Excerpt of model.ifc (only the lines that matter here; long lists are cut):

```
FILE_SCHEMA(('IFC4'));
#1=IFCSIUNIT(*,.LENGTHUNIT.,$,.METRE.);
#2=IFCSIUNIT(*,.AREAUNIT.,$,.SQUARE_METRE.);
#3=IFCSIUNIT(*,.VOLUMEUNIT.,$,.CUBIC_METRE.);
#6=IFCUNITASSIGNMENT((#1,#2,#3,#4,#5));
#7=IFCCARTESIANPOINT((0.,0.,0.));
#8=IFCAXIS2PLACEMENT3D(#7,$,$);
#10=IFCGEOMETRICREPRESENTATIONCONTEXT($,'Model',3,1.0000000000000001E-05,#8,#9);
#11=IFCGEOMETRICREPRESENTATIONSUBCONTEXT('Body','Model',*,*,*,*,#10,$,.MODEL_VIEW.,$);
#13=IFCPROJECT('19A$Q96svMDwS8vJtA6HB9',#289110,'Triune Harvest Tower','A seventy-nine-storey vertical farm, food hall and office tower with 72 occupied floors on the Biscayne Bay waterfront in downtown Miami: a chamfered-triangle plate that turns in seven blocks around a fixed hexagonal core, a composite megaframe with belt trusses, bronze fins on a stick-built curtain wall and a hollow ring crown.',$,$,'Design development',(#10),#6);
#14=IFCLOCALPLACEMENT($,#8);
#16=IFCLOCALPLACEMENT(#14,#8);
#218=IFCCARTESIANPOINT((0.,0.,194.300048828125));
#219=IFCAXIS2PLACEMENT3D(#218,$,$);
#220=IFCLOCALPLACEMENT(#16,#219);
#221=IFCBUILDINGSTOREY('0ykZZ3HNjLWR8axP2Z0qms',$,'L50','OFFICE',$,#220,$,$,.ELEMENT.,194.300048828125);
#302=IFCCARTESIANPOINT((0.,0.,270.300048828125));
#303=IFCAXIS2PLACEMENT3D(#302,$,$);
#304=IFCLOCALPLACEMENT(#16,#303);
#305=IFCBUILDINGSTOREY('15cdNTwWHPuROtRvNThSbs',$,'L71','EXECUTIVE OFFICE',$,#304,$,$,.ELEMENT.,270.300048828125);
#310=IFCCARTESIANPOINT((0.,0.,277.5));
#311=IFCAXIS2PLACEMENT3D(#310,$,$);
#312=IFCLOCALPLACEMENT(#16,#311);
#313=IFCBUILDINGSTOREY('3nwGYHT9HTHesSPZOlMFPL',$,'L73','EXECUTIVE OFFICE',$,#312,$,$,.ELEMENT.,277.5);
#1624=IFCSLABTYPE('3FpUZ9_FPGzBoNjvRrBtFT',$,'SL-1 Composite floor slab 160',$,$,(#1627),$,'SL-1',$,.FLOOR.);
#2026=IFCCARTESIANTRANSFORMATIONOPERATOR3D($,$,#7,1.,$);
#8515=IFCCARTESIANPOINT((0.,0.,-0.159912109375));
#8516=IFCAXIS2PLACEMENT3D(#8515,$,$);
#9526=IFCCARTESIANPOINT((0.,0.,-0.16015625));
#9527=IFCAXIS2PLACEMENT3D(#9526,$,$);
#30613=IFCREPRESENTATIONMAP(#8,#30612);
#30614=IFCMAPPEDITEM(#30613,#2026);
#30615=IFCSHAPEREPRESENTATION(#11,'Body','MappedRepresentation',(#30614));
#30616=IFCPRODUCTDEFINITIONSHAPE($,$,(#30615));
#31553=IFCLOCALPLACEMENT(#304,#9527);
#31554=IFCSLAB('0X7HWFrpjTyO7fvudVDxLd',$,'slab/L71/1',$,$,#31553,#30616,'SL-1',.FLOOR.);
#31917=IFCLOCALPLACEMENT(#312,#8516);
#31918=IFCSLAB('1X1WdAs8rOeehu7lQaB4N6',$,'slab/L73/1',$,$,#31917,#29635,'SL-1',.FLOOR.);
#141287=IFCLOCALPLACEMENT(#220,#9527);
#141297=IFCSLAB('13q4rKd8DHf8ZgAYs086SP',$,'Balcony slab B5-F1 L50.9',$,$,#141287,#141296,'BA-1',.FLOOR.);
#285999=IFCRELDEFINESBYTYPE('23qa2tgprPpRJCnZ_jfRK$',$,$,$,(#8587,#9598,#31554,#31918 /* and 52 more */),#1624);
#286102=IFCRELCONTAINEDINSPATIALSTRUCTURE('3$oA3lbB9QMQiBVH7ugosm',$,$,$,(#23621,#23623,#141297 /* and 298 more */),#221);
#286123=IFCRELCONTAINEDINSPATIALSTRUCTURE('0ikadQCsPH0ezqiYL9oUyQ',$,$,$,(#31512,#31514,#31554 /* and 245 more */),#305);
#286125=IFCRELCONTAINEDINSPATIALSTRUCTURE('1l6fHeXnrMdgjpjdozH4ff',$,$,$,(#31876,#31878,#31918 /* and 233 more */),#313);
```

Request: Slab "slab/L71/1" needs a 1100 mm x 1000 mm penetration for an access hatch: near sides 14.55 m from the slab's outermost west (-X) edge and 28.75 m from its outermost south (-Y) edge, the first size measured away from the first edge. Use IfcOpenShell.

```python
import numpy as np
import ifcopenshell
import ifcopenshell.api.feature
import ifcopenshell.api.geometry
import ifcopenshell.api.root
import ifcopenshell.geom
import ifcopenshell.util.placement
import ifcopenshell.util.representation
import ifcopenshell.util.shape
import ifcopenshell.util.unit

model = ifcopenshell.open("model.ifc")
unit_scale = ifcopenshell.util.unit.calculate_unit_scale(model)
settings = ifcopenshell.geom.settings()


def volume(element):
    """Net volume in cubic metres, openings subtracted."""
    shape = ifcopenshell.geom.create_shape(settings, element)
    return ifcopenshell.util.shape.get_volume(shape.geometry)


slab = model.by_guid("0X7HWFrpjTyO7fvudVDxLd")
before = volume(slab)

# Extent in the slab's own axes, in metres. The edges named are its -X and -Y sides.
slab_shape = ifcopenshell.geom.create_shape(settings, slab)
vertices = ifcopenshell.util.shape.get_vertices(slab_shape.geometry)
x_min, y_min, bottom = vertices.min(axis=0)
top = vertices[:, 2].max()

opening = ifcopenshell.api.root.create_entity(model, ifc_class="IfcOpeningElement", name="Access hatch opening", predefined_type="OPENING")
context = ifcopenshell.util.representation.get_context(model, "Model", "Body", "MODEL_VIEW")
width, depth = 1.1, 1
outline = [(0.0, 0.0), (width, 0.0), (width, depth), (0.0, depth), (0.0, 0.0)]
# Overshoot both faces by 50 mm so the cut is clean.
shape = ifcopenshell.api.geometry.add_slab_representation(
    model, context=context, depth=top - bottom + 0.1, polyline=outline
)
ifcopenshell.api.geometry.assign_representation(model, product=opening, representation=shape)

matrix = ifcopenshell.util.placement.get_local_placement(slab.ObjectPlacement)
matrix[:, 3] = matrix @ np.append(np.array([x_min + 14.55, y_min + 28.75, bottom - 0.05]) / unit_scale, 1.0)
ifcopenshell.api.geometry.edit_object_placement(model, product=opening, matrix=matrix, is_si=False)
ifcopenshell.api.feature.add_feature(model, feature=opening, element=slab)

after = volume(slab)

print(f"slab volume {before:.3f} -> {after:.3f} m3")

model.write("model_rev.ifc")
```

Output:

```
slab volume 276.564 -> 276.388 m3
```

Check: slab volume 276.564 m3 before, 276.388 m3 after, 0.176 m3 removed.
